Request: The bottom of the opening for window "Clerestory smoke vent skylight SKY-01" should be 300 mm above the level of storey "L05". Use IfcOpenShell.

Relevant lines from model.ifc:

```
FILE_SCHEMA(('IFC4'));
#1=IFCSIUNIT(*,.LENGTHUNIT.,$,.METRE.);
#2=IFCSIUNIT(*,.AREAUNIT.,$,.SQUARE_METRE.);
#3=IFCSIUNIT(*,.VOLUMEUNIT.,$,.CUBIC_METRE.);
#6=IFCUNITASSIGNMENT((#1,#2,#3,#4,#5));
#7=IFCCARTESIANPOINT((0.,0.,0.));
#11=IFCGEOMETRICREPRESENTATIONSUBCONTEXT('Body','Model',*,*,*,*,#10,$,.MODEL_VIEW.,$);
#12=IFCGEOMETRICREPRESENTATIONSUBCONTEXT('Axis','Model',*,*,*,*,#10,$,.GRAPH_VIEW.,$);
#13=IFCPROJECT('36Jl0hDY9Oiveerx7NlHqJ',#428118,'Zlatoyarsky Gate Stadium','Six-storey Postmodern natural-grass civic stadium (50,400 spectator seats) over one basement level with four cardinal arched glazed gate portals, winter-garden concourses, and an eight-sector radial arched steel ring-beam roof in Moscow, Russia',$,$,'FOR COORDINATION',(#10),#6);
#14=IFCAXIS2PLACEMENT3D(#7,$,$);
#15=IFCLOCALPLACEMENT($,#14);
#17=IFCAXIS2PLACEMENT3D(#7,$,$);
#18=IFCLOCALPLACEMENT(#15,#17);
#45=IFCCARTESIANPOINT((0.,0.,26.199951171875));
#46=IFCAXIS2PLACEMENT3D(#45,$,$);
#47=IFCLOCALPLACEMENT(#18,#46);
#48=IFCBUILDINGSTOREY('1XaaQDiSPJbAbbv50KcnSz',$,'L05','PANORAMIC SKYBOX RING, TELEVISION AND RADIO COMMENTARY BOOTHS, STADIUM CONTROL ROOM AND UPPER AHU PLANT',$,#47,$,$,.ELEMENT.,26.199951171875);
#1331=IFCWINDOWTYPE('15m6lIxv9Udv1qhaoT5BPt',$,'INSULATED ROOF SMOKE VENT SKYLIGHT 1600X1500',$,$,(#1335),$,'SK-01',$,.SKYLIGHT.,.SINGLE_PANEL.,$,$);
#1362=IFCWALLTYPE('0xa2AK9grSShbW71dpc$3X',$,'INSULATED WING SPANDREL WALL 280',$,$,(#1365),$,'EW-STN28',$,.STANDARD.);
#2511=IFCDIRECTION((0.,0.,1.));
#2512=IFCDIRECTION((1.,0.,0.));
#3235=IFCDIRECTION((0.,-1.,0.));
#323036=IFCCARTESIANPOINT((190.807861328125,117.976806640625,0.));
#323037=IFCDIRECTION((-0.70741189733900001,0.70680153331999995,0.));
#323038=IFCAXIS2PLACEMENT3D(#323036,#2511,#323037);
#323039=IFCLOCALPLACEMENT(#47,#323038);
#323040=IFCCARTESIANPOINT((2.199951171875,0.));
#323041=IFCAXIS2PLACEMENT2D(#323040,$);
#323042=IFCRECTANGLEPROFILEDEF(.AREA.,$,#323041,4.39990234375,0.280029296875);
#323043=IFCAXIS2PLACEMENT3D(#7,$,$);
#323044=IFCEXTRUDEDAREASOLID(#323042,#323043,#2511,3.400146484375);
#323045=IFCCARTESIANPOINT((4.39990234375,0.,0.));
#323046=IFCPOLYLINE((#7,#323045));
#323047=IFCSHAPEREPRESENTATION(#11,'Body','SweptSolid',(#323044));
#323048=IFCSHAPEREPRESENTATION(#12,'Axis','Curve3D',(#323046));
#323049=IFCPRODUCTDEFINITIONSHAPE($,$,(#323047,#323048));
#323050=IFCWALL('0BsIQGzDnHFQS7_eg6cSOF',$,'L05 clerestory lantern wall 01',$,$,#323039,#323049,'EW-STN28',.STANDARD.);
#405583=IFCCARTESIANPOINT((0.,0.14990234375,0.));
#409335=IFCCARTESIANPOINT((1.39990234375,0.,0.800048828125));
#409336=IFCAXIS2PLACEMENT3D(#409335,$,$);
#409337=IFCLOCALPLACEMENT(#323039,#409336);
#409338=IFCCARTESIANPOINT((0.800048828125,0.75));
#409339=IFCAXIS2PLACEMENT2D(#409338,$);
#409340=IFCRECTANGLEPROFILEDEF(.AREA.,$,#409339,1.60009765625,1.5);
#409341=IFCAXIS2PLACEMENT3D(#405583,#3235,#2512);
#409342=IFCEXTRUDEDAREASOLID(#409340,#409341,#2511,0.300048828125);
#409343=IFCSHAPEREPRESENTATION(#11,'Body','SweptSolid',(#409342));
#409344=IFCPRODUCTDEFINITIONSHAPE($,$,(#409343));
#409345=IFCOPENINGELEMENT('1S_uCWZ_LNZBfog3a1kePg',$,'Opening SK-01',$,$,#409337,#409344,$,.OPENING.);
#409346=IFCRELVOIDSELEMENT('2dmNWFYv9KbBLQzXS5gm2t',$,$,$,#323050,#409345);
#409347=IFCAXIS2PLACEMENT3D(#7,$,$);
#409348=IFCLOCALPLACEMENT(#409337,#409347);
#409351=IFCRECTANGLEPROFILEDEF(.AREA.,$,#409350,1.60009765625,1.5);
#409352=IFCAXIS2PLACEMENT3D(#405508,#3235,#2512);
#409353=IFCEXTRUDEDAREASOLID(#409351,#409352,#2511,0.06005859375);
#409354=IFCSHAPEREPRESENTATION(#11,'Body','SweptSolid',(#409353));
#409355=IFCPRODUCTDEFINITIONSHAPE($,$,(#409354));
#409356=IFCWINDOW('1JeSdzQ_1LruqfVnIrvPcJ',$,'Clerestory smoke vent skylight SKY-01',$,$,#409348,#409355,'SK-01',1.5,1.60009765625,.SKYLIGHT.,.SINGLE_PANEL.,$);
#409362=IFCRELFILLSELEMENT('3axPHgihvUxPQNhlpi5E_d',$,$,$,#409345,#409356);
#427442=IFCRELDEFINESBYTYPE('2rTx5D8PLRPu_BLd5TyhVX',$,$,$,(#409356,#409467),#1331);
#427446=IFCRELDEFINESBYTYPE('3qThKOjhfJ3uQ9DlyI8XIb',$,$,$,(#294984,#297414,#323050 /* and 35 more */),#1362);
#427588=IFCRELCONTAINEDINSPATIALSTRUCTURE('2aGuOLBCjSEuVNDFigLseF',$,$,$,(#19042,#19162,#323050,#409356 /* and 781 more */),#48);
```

```python
import numpy as np
import ifcopenshell
import ifcopenshell.api.geometry
import ifcopenshell.geom
import ifcopenshell.util.element
import ifcopenshell.util.placement
import ifcopenshell.util.shape
import ifcopenshell.util.unit

model = ifcopenshell.open("model.ifc")
unit_scale = ifcopenshell.util.unit.calculate_unit_scale(model)

window = model.by_guid("1JeSdzQ_1LruqfVnIrvPcJ")
opening = window.FillsVoids[0].RelatingOpeningElement
storey = ifcopenshell.util.element.get_container(window, ifc_class="IfcBuildingStorey")
level = ifcopenshell.util.placement.get_local_placement(storey.ObjectPlacement)[2, 3]

# The opening's origin need not be at the sill, so measure its lowest point.
shape = ifcopenshell.geom.create_shape(ifcopenshell.geom.settings(), opening)
bottom = ifcopenshell.util.shape.get_shape_bottom_elevation(shape, shape.geometry) / unit_scale
dz = level + 0.3 - bottom

shift = np.array([0.0, 0.0, dz])
# The window is placed relative to its opening, so it follows when the opening moves.
matrix = ifcopenshell.util.placement.get_local_placement(opening.ObjectPlacement)
matrix[:3, 3] += shift
ifcopenshell.api.geometry.edit_object_placement(
    model, product=opening, matrix=matrix, is_si=False, should_transform_children=True
)

print(f"moved by {dz * unit_scale:+.3f} m")

model.write("model_updated.ifc")
```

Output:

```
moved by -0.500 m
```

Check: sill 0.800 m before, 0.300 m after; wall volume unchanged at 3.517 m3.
